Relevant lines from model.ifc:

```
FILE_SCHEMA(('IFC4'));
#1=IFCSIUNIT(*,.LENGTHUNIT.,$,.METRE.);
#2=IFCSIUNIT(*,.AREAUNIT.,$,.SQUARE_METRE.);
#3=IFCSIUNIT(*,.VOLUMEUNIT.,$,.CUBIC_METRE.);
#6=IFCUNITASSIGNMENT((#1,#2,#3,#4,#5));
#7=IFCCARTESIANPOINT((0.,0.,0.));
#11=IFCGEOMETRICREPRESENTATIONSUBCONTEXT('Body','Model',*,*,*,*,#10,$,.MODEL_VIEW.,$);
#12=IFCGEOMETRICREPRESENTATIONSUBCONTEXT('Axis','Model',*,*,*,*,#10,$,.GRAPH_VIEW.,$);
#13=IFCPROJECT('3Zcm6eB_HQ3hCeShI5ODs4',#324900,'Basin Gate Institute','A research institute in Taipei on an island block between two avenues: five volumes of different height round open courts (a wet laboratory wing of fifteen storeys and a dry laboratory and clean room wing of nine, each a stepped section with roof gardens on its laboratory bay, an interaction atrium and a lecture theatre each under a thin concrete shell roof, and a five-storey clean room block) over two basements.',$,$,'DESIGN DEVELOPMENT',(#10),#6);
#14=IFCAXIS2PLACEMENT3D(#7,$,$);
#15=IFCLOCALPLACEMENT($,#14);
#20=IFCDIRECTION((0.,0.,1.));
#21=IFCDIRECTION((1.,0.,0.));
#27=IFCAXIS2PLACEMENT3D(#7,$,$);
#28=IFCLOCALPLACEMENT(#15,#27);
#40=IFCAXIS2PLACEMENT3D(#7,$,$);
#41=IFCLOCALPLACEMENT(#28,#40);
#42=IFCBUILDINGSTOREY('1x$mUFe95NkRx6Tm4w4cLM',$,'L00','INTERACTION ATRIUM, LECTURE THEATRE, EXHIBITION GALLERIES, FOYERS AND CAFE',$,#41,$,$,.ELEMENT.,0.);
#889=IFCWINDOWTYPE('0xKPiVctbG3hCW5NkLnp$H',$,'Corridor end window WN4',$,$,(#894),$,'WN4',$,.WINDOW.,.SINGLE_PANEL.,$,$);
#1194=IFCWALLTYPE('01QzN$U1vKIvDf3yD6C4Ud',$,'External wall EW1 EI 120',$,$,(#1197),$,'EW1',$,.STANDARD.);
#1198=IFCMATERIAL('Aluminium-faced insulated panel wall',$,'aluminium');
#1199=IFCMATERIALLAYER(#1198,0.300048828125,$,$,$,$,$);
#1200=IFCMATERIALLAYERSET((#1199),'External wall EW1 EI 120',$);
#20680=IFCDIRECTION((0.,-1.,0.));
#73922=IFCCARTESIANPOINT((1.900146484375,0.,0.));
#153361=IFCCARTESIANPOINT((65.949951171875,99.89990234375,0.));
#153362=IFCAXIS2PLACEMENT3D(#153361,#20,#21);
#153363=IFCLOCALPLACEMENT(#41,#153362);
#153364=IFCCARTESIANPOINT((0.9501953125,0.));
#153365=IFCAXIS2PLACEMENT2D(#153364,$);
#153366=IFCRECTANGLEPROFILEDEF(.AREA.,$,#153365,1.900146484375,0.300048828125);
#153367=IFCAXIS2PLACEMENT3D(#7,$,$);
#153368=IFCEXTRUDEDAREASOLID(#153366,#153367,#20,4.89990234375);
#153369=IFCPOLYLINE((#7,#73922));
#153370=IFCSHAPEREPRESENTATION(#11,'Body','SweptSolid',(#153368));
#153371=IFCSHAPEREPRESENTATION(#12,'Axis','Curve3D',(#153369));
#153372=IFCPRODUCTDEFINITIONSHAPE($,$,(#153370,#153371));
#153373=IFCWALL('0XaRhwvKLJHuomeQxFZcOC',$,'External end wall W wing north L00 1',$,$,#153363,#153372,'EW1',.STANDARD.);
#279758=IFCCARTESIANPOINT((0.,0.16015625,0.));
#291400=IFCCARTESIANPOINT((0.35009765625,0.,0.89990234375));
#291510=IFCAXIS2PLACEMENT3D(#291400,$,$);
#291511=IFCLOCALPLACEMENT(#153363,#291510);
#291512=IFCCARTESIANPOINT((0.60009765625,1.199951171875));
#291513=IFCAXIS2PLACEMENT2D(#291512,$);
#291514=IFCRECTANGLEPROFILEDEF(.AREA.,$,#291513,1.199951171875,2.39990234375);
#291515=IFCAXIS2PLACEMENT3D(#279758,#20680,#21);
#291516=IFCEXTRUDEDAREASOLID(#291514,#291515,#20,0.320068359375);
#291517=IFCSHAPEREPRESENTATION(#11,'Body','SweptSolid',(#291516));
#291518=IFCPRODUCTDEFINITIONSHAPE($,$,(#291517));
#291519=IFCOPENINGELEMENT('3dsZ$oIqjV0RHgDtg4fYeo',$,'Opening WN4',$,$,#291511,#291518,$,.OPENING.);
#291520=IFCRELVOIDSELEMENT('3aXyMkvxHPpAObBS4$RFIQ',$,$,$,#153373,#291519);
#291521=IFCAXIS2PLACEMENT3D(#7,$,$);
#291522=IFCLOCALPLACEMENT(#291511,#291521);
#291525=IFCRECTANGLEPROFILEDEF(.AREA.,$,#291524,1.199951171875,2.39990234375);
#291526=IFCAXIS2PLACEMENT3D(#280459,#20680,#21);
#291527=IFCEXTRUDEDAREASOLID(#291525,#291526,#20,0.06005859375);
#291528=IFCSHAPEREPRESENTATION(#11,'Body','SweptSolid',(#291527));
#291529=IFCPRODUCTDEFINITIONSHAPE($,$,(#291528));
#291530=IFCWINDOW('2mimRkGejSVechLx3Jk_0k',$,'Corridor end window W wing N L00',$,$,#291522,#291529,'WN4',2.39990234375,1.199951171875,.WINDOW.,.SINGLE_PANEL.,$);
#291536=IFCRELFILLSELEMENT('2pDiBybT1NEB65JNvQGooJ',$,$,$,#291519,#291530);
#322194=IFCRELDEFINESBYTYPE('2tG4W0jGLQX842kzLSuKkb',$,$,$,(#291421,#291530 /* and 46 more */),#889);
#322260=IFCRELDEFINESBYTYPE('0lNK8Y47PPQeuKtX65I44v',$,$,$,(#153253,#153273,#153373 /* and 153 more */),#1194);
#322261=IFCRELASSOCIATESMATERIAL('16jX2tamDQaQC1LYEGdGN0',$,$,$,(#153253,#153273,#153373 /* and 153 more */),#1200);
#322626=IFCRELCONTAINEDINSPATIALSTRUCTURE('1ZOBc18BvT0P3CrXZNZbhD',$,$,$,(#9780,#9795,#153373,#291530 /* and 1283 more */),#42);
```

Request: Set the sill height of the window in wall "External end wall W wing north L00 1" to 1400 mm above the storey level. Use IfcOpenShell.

```python
import numpy as np
import ifcopenshell
import ifcopenshell.api.geometry
import ifcopenshell.geom
import ifcopenshell.util.element
import ifcopenshell.util.placement
import ifcopenshell.util.shape
import ifcopenshell.util.unit

model = ifcopenshell.open("model.ifc")
unit_scale = ifcopenshell.util.unit.calculate_unit_scale(model)

window = model.by_guid("2mimRkGejSVechLx3Jk_0k")
opening = window.FillsVoids[0].RelatingOpeningElement
storey = ifcopenshell.util.element.get_container(window, ifc_class="IfcBuildingStorey")
level = ifcopenshell.util.placement.get_local_placement(storey.ObjectPlacement)[2, 3]

# The opening's origin need not be at the sill, so measure its lowest point.
shape = ifcopenshell.geom.create_shape(ifcopenshell.geom.settings(), opening)
bottom = ifcopenshell.util.shape.get_shape_bottom_elevation(shape, shape.geometry) / unit_scale
dz = level + 1.4 / unit_scale - bottom

shift = np.array([0.0, 0.0, dz])
# The window is placed relative to its opening, so it follows when the opening moves.
matrix = ifcopenshell.util.placement.get_local_placement(opening.ObjectPlacement)
matrix[:3, 3] += shift
ifcopenshell.api.geometry.edit_object_placement(
    model, product=opening, matrix=matrix, is_si=False, should_transform_children=True
)

print(f"moved by {dz * unit_scale:+.3f} m")

model.write("model_edited.ifc")
```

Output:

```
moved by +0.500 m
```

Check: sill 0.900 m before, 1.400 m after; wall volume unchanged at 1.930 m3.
